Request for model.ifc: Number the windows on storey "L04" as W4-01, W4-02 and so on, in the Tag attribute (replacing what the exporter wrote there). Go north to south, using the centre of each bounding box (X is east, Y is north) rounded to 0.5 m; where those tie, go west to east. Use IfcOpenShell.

First a look at what the model holds.

```python
import ifcopenshell
import ifcopenshell.util.element
import ifcopenshell.util.placement

model = ifcopenshell.open("model.ifc")
print(model.schema)
storey = next(s for s in model.by_type("IfcBuildingStorey") if s.Name == "L04")
windows = [e for e in ifcopenshell.util.element.get_decomposition(storey) if e.is_a("IfcWindow")]
for e in sorted(windows, key=lambda e: e.id()):
    origin = ifcopenshell.util.placement.get_local_placement(e.ObjectPlacement)[:3, 3]
    print(e.id(), e.Tag, e.Name, origin.round(2) + 0.0, sep=" | ")
```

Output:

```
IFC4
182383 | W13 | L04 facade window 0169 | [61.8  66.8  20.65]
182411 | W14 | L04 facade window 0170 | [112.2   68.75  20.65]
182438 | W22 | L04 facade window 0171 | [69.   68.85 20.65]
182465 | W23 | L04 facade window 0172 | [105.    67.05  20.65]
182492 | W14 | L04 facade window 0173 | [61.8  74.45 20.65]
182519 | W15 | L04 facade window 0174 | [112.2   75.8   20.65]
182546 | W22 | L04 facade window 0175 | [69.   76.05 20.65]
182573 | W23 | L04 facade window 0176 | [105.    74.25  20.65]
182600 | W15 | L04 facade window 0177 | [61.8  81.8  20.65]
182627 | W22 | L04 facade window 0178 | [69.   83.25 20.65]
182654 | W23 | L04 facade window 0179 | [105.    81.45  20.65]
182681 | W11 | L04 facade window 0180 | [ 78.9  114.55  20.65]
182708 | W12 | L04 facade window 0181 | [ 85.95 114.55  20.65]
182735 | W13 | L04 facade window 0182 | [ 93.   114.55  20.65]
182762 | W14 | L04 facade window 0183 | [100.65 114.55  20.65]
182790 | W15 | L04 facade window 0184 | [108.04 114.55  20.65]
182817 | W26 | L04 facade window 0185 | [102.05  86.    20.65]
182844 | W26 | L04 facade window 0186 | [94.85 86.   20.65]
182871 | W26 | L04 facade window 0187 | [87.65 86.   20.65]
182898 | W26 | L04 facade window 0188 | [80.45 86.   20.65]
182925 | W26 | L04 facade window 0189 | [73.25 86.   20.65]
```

```python
import ifcopenshell
import ifcopenshell.geom
import ifcopenshell.util.element
import ifcopenshell.util.shape

model = ifcopenshell.open("model.ifc")
settings = ifcopenshell.geom.settings()
settings.set("use-world-coords", True)


def centre(element):
    shape = ifcopenshell.geom.create_shape(settings, element)
    return ifcopenshell.util.shape.get_bbox_centroid(shape.geometry)


storey = next(s for s in model.by_type("IfcBuildingStorey") if s.Name == "L04")
windows = [e for e in ifcopenshell.util.element.get_decomposition(storey) if e.is_a("IfcWindow")]

# Insertion points can sit at a corner or the storey origin, so sort by the geometry (in metres).
centres = {e: centre(e) for e in windows}
windows.sort(key=lambda e: (-round(centres[e][1] / 0.5), centres[e][0]))

for i, e in enumerate(windows, start=1):
    number = f"W4-{i:02d}"
    e.Tag = number
    print(e.id(), number)

model.write("model-out.ifc")
```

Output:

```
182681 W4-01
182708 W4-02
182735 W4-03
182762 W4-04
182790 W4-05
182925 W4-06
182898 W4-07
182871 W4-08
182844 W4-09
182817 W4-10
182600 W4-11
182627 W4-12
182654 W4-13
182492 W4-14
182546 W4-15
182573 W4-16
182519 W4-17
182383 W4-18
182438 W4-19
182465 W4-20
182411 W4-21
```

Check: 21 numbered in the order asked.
